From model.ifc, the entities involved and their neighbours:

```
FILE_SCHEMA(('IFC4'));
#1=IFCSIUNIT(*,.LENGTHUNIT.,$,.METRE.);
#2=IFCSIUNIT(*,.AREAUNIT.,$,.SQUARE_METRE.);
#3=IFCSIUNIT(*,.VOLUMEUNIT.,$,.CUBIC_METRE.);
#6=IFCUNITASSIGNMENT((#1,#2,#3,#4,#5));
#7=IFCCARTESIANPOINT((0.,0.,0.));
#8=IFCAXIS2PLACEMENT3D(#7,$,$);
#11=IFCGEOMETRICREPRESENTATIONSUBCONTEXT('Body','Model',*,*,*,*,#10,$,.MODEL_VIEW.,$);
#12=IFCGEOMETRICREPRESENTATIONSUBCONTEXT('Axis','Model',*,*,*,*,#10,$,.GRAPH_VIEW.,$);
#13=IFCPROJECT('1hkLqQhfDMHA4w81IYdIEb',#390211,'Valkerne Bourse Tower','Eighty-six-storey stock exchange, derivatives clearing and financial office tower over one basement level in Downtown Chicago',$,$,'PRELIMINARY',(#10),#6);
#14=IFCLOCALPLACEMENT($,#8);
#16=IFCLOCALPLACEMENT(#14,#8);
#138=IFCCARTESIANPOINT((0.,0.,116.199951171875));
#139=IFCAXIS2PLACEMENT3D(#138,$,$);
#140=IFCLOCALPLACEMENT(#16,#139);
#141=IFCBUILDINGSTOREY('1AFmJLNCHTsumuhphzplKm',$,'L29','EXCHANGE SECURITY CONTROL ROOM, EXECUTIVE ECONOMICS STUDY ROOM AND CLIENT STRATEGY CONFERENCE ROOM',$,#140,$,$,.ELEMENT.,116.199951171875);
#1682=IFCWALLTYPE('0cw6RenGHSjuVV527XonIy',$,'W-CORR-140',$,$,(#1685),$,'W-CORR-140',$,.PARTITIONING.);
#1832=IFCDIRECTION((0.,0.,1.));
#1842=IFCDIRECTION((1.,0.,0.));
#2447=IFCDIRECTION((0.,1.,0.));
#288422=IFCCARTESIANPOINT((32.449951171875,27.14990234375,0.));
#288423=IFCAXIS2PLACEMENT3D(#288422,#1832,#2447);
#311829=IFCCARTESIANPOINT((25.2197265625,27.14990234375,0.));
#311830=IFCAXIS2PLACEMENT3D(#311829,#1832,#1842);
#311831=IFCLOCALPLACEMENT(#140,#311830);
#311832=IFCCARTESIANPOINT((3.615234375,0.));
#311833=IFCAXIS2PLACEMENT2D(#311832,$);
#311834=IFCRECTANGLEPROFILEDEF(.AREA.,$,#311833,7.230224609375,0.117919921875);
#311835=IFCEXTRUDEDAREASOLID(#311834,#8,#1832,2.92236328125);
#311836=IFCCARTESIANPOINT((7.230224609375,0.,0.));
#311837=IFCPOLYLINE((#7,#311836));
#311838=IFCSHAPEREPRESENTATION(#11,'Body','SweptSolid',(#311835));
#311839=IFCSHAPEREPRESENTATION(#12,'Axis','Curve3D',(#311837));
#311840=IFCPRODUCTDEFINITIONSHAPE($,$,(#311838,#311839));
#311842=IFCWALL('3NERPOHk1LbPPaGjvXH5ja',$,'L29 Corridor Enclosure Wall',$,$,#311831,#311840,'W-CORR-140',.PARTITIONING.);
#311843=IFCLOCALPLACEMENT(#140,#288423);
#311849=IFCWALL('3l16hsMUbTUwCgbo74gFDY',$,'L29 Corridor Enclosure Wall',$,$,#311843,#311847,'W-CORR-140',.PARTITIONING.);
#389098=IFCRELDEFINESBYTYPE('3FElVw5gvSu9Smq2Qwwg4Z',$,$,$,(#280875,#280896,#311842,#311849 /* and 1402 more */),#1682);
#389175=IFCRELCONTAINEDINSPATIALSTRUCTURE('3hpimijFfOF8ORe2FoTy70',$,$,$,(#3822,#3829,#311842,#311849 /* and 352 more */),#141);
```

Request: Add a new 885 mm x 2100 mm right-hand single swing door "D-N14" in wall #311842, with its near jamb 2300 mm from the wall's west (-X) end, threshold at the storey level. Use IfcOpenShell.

```python
import numpy as np
import ifcopenshell
import ifcopenshell.api.feature
import ifcopenshell.api.geometry
import ifcopenshell.api.root
import ifcopenshell.api.spatial
import ifcopenshell.geom
import ifcopenshell.util.element
import ifcopenshell.util.placement
import ifcopenshell.util.representation
import ifcopenshell.util.shape
import ifcopenshell.util.unit

model = ifcopenshell.open("model.ifc")
unit_scale = ifcopenshell.util.unit.calculate_unit_scale(model)
settings = ifcopenshell.geom.settings()


def volume(element):
    """Net volume in cubic metres, openings subtracted."""
    shape = ifcopenshell.geom.create_shape(settings, element)
    return ifcopenshell.util.shape.get_volume(shape.geometry)


wall = model.by_guid("3NERPOHk1LbPPaGjvXH5ja")
storey = ifcopenshell.util.element.get_container(wall, ifc_class="IfcBuildingStorey")
context = ifcopenshell.util.representation.get_context(model, "Model", "Body", "MODEL_VIEW")
before = volume(wall)

width, height, from_end, sill = 0.885, 2.1, 2.3, 0.0  # metres

# The wall runs along its own X axis, and the end named is its -X end.
wall_shape = ifcopenshell.geom.create_shape(settings, wall)
x, y, z = ifcopenshell.util.shape.get_vertices(wall_shape.geometry).T
start = x.min() + from_end
face, thickness = float(y.min()), float(y.max() - y.min())
wall_matrix = ifcopenshell.util.placement.get_local_placement(wall.ObjectPlacement)
level = ifcopenshell.util.placement.get_local_placement(storey.ObjectPlacement)[2, 3]


def in_wall(x, y):
    """Placement at x, y metres in the wall's axes, at sill height."""
    matrix = wall_matrix.copy()
    matrix[:, 3] = wall_matrix @ np.array([x / unit_scale, y / unit_scale, 0.0, 1.0])
    matrix[2, 3] = level + sill / unit_scale
    return matrix


# Opening: a box that overshoots both wall faces by 50 mm.
opening = ifcopenshell.api.root.create_entity(model, ifc_class="IfcOpeningElement", predefined_type="OPENING")
box = ifcopenshell.api.geometry.add_wall_representation(
    model, context=context, length=width, height=height, thickness=thickness + 0.1
)
ifcopenshell.api.geometry.assign_representation(model, product=opening, representation=box)
ifcopenshell.api.geometry.edit_object_placement(model, product=opening, matrix=in_wall(start, face - 0.05), is_si=False)
ifcopenshell.api.feature.add_feature(model, feature=opening, element=wall)

door = ifcopenshell.api.root.create_entity(model, ifc_class="IfcDoor", name="D-N14", predefined_type="DOOR")
door.OverallWidth, door.OverallHeight = width / unit_scale, height / unit_scale
door.OperationType = "SINGLE_SWING_RIGHT"
body = ifcopenshell.api.geometry.add_door_representation(
    model,
    context=context,
    overall_width=door.OverallWidth,
    overall_height=door.OverallHeight,
    operation_type="SINGLE_SWING_RIGHT",
    lining_properties={"LiningDepth": thickness / unit_scale, "ThresholdDepth": thickness / unit_scale},
)
ifcopenshell.api.geometry.assign_representation(model, product=door, representation=body)
ifcopenshell.api.spatial.assign_container(model, products=[door], relating_structure=storey)
ifcopenshell.api.feature.add_filling(model, opening=opening, element=door)

# The lining spans the wall, so the door starts at the wall face.
ifcopenshell.api.geometry.edit_object_placement(model, product=door, matrix=in_wall(start, face), is_si=False)

after = volume(wall)

print(f"wall volume {before:.3f} -> {after:.3f} m3")

model.write("model_edited.ifc")
```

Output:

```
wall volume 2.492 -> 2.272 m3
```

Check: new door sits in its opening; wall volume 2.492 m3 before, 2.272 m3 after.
